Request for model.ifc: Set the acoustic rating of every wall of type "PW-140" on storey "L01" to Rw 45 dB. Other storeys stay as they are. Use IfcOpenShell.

First a look at what the model holds.

```python
import ifcopenshell
import ifcopenshell.util.element

model = ifcopenshell.open("model.ifc")
print(model.schema)
storey = next(s for s in model.by_type("IfcBuildingStorey") if s.Name == "L01")
walls = [e for e in ifcopenshell.util.element.get_decomposition(storey) if e.is_a("IfcWall")]
seen = {}
for e in walls:
    element_type = ifcopenshell.util.element.get_type(e)
    key = (element_type.Name if element_type != e and element_type else None, ifcopenshell.util.element.get_pset(e, "Pset_WallCommon", "AcousticRating"))
    seen[key] = seen.get(key, 0) + 1
for (name, value), count in sorted(seen.items(), key=str):
    print(count, "x", name, "|", value)
```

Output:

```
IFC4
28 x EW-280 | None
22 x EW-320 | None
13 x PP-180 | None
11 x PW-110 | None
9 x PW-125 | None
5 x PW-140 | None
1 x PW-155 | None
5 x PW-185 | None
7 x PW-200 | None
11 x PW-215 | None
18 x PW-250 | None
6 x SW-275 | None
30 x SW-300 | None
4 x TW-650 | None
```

```python
import ifcopenshell
import ifcopenshell.api.pset
import ifcopenshell.util.element

model = ifcopenshell.open("model.ifc")

storey = next(s for s in model.by_type("IfcBuildingStorey") if s.Name == "L01")
walls = [e for e in ifcopenshell.util.element.get_decomposition(storey) if e.is_a("IfcWall")]

count = 0
for e in walls:
    element_type = ifcopenshell.util.element.get_type(e)
    if element_type in (None, e) or element_type.Name != "PW-140":
        continue
    # add_pset returns the element's existing set when there is one.
    pset = ifcopenshell.api.pset.add_pset(model, product=e, name="Pset_WallCommon")
    ifcopenshell.api.pset.edit_pset(model, pset=pset, properties={"AcousticRating": "Rw 45 dB"})
    count += 1

print(count, "walls updated")

model.write("model_edited.ifc")
```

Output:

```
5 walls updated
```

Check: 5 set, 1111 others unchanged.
